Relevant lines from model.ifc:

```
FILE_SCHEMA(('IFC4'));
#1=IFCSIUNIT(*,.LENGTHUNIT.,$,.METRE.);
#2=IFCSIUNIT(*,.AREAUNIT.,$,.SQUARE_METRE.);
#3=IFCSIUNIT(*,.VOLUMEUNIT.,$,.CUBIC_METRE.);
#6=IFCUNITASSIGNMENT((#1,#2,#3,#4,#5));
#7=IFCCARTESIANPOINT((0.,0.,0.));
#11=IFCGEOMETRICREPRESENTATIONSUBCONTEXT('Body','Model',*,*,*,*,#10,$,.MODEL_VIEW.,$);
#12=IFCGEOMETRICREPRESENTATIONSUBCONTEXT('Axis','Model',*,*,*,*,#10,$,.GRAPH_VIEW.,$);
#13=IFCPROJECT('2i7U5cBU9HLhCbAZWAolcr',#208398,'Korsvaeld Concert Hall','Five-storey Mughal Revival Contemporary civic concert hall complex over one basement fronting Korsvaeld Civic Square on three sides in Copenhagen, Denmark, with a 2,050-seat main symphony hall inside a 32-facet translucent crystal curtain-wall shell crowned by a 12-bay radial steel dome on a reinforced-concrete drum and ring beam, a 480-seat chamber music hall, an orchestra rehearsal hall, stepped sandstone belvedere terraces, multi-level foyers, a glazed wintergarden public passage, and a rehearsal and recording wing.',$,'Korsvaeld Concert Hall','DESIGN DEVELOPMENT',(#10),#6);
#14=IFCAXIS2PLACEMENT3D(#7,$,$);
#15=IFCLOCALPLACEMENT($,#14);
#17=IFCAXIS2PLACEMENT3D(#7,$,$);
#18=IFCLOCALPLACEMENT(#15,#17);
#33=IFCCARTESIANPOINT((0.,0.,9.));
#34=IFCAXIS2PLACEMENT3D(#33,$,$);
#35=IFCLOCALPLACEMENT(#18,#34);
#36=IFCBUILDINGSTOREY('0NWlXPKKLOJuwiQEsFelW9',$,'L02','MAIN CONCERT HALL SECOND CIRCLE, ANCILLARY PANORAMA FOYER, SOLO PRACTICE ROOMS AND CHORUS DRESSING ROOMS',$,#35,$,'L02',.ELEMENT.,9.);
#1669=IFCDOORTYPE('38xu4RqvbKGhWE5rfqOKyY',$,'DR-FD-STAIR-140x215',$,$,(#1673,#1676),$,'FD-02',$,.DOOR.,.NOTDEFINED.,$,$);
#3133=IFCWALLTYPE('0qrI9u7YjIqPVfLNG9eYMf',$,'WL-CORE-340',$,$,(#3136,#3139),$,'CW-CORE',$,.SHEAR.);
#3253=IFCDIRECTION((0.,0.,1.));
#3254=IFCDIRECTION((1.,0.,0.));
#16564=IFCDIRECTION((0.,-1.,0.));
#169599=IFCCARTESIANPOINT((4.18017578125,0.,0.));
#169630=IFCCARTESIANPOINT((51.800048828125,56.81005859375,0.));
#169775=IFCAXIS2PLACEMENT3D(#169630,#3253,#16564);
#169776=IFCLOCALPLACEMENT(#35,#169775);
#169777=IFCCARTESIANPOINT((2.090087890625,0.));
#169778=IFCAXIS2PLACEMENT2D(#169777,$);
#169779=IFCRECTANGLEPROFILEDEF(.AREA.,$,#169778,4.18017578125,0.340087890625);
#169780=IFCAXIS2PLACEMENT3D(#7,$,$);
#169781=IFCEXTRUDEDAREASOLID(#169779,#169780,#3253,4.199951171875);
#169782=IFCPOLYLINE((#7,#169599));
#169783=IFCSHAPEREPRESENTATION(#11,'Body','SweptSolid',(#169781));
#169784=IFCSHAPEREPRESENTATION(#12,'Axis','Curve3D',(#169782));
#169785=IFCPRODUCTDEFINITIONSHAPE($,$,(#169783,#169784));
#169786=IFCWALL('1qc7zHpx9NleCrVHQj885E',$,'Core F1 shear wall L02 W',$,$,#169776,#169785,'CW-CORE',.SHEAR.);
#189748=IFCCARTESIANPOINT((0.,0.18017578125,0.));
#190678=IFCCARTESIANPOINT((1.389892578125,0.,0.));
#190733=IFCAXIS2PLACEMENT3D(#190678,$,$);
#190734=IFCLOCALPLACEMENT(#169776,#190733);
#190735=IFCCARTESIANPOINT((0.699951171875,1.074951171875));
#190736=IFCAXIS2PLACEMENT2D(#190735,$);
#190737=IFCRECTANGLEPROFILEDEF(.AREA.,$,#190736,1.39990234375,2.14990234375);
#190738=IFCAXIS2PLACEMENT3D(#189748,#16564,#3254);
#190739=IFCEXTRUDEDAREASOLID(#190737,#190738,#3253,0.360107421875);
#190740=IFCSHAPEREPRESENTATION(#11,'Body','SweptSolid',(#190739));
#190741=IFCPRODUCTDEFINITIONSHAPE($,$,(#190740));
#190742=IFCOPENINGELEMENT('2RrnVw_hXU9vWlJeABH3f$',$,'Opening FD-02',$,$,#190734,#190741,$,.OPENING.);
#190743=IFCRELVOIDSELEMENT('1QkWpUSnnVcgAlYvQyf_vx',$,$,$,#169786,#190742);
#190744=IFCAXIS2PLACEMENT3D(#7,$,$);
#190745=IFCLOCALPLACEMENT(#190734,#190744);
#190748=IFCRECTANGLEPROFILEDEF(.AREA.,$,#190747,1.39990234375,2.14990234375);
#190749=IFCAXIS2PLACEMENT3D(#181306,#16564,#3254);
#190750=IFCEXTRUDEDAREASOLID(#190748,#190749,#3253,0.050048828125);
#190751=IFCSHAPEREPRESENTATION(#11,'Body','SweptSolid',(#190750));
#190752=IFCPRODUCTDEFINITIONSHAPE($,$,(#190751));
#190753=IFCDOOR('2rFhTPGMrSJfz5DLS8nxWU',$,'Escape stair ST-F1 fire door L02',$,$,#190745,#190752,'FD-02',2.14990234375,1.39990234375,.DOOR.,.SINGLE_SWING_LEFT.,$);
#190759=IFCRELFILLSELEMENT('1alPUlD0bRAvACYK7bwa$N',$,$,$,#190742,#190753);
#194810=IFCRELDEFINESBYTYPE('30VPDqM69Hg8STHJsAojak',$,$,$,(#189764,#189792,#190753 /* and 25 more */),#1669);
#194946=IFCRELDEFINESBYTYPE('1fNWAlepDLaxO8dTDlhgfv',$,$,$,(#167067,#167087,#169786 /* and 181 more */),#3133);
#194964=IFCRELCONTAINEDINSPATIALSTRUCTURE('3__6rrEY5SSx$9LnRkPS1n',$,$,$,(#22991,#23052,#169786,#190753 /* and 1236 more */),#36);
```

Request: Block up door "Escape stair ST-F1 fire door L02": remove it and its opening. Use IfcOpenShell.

```python
import ifcopenshell
import ifcopenshell.api.feature
import ifcopenshell.api.root
import ifcopenshell.geom
import ifcopenshell.util.shape

model = ifcopenshell.open("model.ifc")
settings = ifcopenshell.geom.settings()


def volume(element):
    """Net volume in cubic metres, openings subtracted."""
    shape = ifcopenshell.geom.create_shape(settings, element)
    return ifcopenshell.util.shape.get_volume(shape.geometry)


door = model.by_id(190753)
opening = door.FillsVoids[0].RelatingOpeningElement
wall = opening.VoidsElements[0].RelatingBuildingElement
before = volume(wall)

ifcopenshell.api.root.remove_product(model, product=door)
ifcopenshell.api.feature.remove_feature(model, feature=opening)

after = volume(wall)

print(f"wall volume {before:.3f} -> {after:.3f} m3")

model.write("model_updated.ifc")
```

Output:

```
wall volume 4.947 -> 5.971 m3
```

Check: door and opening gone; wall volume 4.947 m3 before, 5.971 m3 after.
